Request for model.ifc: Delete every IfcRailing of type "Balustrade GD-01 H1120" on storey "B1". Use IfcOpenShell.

First a look at what the model holds.

```python
import ifcopenshell
import ifcopenshell.util.element

model = ifcopenshell.open("model.ifc")
print(model.schema)
storey = next(s for s in model.by_type("IfcBuildingStorey") if s.Name == "B1")
railings = [e for e in ifcopenshell.util.element.get_decomposition(storey) if e.is_a("IfcRailing")]
seen = {}
for e in railings:
    element_type = ifcopenshell.util.element.get_type(e)
    name = element_type.Name if element_type not in (None, e) else None
    seen[name] = seen.get(name, 0) + 1
for name, count in sorted(seen.items(), key=str):
    print(count, "x", name)
```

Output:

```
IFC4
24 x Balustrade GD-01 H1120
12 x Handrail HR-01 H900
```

```python
import ifcopenshell
import ifcopenshell.api.root
import ifcopenshell.util.element

model = ifcopenshell.open("model.ifc")

storey = next(s for s in model.by_type("IfcBuildingStorey") if s.Name == "B1")
railings = [e for e in ifcopenshell.util.element.get_decomposition(storey) if e.is_a("IfcRailing")]
targets = [e for e in railings if (t := ifcopenshell.util.element.get_type(e)) not in (None, e) and t.Name == "Balustrade GD-01 H1120"]

for e in targets:
    ifcopenshell.api.root.remove_product(model, product=e)
print(len(targets), "removed")

model.write("model_updated.ifc")
```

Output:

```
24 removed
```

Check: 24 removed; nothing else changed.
